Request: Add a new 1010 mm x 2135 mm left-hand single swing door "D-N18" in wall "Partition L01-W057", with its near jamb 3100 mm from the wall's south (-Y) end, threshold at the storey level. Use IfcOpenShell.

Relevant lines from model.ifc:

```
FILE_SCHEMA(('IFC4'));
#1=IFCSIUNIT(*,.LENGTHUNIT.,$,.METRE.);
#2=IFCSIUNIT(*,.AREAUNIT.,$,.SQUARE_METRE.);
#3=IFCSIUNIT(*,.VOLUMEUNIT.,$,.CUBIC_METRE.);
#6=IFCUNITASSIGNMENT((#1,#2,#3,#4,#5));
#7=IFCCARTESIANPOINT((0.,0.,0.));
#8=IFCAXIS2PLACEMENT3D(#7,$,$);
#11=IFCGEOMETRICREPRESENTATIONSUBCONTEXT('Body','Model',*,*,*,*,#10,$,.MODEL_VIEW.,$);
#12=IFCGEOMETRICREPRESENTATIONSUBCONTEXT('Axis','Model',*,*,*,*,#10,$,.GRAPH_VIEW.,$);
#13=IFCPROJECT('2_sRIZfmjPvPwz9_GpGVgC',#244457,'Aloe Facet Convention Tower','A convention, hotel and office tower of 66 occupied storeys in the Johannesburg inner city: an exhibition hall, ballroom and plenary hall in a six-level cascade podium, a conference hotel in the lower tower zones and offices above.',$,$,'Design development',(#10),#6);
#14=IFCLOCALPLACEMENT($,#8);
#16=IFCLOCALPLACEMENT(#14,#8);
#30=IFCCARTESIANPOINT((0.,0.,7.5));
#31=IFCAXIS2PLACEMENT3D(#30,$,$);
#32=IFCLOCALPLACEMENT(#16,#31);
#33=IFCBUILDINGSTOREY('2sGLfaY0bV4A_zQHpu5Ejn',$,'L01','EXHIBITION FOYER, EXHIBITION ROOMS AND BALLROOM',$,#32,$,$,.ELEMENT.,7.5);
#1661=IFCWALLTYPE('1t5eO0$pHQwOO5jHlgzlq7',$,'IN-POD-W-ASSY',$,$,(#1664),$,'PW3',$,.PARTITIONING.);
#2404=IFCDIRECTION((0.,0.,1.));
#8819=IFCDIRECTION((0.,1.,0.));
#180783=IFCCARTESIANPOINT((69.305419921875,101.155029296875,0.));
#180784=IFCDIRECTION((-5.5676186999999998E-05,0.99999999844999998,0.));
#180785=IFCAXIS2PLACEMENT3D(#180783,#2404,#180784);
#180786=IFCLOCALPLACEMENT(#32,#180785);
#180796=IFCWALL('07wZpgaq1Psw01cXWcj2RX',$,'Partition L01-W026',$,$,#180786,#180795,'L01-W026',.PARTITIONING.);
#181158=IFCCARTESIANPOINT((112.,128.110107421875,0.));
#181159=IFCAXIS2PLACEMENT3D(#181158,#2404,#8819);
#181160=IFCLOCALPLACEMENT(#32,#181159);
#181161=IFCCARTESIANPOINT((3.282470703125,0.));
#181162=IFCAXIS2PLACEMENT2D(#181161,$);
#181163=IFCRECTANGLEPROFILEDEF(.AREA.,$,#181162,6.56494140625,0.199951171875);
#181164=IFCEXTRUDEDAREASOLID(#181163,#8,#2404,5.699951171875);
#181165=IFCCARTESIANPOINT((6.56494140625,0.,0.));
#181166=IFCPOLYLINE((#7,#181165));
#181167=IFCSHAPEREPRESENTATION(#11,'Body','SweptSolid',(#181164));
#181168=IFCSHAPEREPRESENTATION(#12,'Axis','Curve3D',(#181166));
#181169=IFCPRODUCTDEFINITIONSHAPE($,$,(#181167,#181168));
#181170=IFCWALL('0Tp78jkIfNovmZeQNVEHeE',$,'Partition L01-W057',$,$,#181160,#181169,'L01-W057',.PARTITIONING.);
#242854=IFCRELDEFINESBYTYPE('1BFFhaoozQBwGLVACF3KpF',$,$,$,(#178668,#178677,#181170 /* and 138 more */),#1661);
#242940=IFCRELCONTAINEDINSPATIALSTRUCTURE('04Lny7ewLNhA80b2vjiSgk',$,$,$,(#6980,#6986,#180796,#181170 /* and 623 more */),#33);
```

```python
import numpy as np
import ifcopenshell
import ifcopenshell.api.feature
import ifcopenshell.api.geometry
import ifcopenshell.api.root
import ifcopenshell.api.spatial
import ifcopenshell.geom
import ifcopenshell.util.element
import ifcopenshell.util.placement
import ifcopenshell.util.representation
import ifcopenshell.util.shape
import ifcopenshell.util.unit

model = ifcopenshell.open("model.ifc")
unit_scale = ifcopenshell.util.unit.calculate_unit_scale(model)
settings = ifcopenshell.geom.settings()


def volume(element):
    """Net volume in cubic metres, openings subtracted."""
    shape = ifcopenshell.geom.create_shape(settings, element)
    return ifcopenshell.util.shape.get_volume(shape.geometry)


wall = model.by_guid("0Tp78jkIfNovmZeQNVEHeE")
storey = ifcopenshell.util.element.get_container(wall, ifc_class="IfcBuildingStorey")
context = ifcopenshell.util.representation.get_context(model, "Model", "Body", "MODEL_VIEW")
before = volume(wall)

width, height, from_end, sill = 1.01, 2.135, 3.1, 0.0  # metres

# The wall runs along its own X axis, and the end named is its -X end.
wall_shape = ifcopenshell.geom.create_shape(settings, wall)
x, y, z = ifcopenshell.util.shape.get_vertices(wall_shape.geometry).T
start = x.min() + from_end
face, thickness = float(y.min()), float(y.max() - y.min())
wall_matrix = ifcopenshell.util.placement.get_local_placement(wall.ObjectPlacement)
level = ifcopenshell.util.placement.get_local_placement(storey.ObjectPlacement)[2, 3]


def in_wall(x, y):
    """Placement at x, y metres in the wall's axes, at sill height."""
    matrix = wall_matrix.copy()
    matrix[:, 3] = wall_matrix @ np.array([x / unit_scale, y / unit_scale, 0.0, 1.0])
    matrix[2, 3] = level + sill / unit_scale
    return matrix


# Opening: a box that overshoots both wall faces by 50 mm.
opening = ifcopenshell.api.root.create_entity(model, ifc_class="IfcOpeningElement", predefined_type="OPENING")
box = ifcopenshell.api.geometry.add_wall_representation(
    model, context=context, length=width, height=height, thickness=thickness + 0.1
)
ifcopenshell.api.geometry.assign_representation(model, product=opening, representation=box)
ifcopenshell.api.geometry.edit_object_placement(model, product=opening, matrix=in_wall(start, face - 0.05), is_si=False)
ifcopenshell.api.feature.add_feature(model, feature=opening, element=wall)

door = ifcopenshell.api.root.create_entity(model, ifc_class="IfcDoor", name="D-N18", predefined_type="DOOR")
door.OverallWidth, door.OverallHeight = width / unit_scale, height / unit_scale
door.OperationType = "SINGLE_SWING_LEFT"
body = ifcopenshell.api.geometry.add_door_representation(
    model,
    context=context,
    overall_width=door.OverallWidth,
    overall_height=door.OverallHeight,
    operation_type="SINGLE_SWING_LEFT",
    lining_properties={"LiningDepth": thickness / unit_scale, "ThresholdDepth": thickness / unit_scale},
)
ifcopenshell.api.geometry.assign_representation(model, product=door, representation=body)
ifcopenshell.api.spatial.assign_container(model, products=[door], relating_structure=storey)
ifcopenshell.api.feature.add_filling(model, opening=opening, element=door)

# The lining spans the wall, so the door starts at the wall face.
ifcopenshell.api.geometry.edit_object_placement(model, product=door, matrix=in_wall(start, face), is_si=False)

after = volume(wall)

print(f"wall volume {before:.3f} -> {after:.3f} m3")

model.write("model_edited.ifc")
```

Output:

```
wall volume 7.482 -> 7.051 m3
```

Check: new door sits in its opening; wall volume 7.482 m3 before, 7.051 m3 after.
